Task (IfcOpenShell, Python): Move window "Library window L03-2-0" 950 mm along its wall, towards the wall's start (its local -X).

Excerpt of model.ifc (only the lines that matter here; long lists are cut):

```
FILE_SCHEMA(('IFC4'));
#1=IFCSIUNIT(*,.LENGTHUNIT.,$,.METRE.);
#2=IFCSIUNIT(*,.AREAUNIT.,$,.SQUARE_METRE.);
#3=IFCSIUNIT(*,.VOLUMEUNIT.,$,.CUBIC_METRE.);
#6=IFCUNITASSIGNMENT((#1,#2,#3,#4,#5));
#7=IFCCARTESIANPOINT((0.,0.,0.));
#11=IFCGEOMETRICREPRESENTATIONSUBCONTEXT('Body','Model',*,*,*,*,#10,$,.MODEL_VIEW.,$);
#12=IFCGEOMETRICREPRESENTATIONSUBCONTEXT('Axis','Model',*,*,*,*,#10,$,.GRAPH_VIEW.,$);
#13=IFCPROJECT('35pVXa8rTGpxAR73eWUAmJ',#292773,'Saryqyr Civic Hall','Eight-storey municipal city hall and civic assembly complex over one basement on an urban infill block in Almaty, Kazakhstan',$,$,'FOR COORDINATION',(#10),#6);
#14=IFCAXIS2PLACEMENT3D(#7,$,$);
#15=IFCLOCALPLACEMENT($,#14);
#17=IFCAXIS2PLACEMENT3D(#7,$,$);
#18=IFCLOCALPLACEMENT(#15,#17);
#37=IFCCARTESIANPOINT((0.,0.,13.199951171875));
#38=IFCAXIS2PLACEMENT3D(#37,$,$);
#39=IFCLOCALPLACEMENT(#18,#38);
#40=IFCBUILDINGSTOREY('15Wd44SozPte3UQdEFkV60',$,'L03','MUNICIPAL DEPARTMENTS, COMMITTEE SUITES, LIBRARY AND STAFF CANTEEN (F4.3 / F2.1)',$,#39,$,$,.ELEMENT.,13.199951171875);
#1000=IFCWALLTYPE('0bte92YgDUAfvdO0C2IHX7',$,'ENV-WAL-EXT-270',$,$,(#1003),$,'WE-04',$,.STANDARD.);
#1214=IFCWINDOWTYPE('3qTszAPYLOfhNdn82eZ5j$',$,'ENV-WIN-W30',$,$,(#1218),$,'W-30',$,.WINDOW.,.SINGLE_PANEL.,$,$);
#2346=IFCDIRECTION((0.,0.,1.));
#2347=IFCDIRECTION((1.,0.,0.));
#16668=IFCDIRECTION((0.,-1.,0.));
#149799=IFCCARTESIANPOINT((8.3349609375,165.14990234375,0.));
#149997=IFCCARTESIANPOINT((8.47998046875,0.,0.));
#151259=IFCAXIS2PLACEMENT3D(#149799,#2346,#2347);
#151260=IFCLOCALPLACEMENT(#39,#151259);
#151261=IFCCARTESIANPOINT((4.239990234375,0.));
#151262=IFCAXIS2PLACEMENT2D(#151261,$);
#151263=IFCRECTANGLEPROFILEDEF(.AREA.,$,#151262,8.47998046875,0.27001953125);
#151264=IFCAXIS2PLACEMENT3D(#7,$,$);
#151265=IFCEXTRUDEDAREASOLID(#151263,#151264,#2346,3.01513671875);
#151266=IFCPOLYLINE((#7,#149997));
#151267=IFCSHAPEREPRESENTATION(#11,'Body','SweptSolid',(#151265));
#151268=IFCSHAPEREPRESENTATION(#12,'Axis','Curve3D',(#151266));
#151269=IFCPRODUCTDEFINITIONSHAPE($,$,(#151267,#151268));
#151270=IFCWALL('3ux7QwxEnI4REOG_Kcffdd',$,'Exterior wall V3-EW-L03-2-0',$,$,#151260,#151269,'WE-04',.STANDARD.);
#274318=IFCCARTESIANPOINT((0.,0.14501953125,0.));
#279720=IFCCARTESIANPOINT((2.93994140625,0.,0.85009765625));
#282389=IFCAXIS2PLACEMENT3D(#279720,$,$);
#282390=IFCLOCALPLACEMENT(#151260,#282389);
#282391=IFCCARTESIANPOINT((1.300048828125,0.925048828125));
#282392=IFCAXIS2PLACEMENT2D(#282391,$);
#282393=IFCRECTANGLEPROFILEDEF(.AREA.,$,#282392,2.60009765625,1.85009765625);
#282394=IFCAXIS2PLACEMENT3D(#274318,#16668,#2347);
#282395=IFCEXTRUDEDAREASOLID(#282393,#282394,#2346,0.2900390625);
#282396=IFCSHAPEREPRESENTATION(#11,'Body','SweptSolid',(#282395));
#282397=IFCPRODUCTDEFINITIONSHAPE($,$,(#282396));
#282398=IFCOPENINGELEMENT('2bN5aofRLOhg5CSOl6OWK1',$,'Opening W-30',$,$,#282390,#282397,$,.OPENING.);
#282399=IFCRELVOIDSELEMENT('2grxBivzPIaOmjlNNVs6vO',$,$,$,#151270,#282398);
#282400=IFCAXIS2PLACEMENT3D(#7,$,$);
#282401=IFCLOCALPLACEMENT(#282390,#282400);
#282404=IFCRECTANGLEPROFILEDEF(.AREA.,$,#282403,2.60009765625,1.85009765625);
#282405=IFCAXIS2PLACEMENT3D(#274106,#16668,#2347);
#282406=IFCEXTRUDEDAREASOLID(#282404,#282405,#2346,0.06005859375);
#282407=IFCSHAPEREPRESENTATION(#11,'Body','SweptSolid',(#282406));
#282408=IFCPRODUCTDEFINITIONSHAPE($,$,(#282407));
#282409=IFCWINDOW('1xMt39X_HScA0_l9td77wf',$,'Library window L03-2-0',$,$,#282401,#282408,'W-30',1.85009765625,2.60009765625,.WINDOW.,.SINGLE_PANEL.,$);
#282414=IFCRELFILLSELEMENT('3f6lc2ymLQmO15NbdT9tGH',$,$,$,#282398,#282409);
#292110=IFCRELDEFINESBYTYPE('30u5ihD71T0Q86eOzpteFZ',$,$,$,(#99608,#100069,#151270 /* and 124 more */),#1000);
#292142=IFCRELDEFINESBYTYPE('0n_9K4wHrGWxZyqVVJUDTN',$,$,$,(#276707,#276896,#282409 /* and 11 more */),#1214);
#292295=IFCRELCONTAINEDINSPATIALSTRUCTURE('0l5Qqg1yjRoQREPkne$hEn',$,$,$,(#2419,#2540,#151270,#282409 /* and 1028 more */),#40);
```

```python
import ifcopenshell
import ifcopenshell.api.geometry
import ifcopenshell.util.placement
import ifcopenshell.util.unit

model = ifcopenshell.open("model.ifc")
unit_scale = ifcopenshell.util.unit.calculate_unit_scale(model)

window = model.by_guid("1xMt39X_HScA0_l9td77wf")
opening = window.FillsVoids[0].RelatingOpeningElement
wall = opening.VoidsElements[0].RelatingBuildingElement

wall_matrix = ifcopenshell.util.placement.get_local_placement(wall.ObjectPlacement)
shift = wall_matrix[:3, 0] * -0.95 / unit_scale
before = ifcopenshell.util.placement.get_local_placement(window.ObjectPlacement)[:3, 3].copy()

# The window is placed relative to its opening, so it follows when the opening moves.
matrix = ifcopenshell.util.placement.get_local_placement(opening.ObjectPlacement)
matrix[:3, 3] += shift
ifcopenshell.api.geometry.edit_object_placement(
    model, product=opening, matrix=matrix, is_si=False, should_transform_children=True
)

after = ifcopenshell.util.placement.get_local_placement(window.ObjectPlacement)[:3, 3]
print("window moved by", (after - before).round(3) + 0.0)

model.write("model_updated.ifc")
```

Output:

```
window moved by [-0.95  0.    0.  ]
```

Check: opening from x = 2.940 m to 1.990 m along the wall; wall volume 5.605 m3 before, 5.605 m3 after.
